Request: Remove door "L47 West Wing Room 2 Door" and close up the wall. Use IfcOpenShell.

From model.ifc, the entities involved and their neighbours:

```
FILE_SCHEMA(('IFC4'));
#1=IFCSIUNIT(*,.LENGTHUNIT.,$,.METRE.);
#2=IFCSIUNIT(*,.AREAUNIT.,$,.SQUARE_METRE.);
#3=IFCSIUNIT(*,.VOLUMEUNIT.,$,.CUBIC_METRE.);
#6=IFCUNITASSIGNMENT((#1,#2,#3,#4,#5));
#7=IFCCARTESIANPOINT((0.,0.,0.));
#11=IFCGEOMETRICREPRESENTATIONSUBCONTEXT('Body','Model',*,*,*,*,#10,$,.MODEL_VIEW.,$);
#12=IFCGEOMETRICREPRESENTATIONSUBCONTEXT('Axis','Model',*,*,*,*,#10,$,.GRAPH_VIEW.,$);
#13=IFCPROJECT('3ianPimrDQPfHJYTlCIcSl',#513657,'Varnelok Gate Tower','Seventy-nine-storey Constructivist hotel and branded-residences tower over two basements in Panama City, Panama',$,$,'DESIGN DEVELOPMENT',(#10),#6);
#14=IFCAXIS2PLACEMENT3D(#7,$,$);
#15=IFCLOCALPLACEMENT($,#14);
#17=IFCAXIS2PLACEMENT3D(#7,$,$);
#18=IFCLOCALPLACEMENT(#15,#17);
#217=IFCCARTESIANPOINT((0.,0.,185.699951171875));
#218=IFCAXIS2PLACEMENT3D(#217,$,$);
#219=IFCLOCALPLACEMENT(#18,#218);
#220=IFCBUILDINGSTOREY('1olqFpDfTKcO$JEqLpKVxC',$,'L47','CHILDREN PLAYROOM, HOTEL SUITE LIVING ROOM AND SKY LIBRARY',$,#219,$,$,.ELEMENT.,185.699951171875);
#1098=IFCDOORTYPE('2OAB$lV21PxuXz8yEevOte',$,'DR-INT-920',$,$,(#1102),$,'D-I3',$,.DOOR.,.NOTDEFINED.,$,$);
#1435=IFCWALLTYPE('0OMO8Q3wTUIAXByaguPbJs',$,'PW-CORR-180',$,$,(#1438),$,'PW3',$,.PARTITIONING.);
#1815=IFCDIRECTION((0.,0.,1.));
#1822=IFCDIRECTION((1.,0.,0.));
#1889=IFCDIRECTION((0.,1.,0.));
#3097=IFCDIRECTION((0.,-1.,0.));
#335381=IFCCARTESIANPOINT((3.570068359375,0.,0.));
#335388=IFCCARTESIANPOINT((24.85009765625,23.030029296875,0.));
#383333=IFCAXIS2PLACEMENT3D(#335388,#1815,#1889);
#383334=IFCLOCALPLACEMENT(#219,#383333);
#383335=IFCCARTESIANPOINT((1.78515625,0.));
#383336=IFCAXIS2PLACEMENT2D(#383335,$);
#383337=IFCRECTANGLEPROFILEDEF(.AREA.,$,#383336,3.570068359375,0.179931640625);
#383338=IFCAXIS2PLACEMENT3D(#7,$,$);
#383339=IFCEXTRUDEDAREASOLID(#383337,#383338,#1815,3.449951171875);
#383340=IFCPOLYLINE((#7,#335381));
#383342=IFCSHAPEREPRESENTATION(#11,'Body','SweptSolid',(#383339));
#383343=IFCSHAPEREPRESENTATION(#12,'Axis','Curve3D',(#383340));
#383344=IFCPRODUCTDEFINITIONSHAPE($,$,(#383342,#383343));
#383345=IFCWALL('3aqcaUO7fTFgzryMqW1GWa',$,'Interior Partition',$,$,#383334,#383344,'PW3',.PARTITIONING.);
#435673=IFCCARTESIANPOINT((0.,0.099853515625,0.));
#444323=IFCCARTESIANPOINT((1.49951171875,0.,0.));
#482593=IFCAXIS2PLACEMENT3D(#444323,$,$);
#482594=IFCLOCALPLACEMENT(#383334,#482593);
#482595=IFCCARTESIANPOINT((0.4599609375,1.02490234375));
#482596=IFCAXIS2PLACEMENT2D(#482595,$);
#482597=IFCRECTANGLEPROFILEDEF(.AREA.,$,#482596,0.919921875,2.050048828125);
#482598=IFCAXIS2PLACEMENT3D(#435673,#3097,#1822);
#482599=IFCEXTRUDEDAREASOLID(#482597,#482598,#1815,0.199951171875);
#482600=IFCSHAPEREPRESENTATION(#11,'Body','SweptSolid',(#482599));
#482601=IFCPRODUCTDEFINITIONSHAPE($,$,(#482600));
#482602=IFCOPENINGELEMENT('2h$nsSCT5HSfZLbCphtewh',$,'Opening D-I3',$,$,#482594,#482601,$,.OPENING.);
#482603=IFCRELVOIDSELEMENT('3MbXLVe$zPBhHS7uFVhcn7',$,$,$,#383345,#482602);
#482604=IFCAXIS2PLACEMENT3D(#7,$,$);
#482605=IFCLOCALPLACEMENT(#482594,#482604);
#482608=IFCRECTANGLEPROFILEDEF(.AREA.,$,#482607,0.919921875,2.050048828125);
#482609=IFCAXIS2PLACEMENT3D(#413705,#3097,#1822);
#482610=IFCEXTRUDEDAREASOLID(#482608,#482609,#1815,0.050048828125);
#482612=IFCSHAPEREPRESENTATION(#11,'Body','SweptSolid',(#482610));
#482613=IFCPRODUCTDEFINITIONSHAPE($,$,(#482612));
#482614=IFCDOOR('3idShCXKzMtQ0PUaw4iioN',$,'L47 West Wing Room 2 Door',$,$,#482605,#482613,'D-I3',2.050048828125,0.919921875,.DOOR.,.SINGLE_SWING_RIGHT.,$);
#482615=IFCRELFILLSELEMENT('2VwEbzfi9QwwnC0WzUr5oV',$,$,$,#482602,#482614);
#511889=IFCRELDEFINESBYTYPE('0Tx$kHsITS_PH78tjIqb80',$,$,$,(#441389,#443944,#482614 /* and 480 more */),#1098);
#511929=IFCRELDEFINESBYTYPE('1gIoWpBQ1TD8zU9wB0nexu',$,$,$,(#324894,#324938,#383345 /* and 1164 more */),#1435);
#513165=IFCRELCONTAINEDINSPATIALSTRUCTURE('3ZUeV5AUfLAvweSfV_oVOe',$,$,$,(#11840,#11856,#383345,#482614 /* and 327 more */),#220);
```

```python
import ifcopenshell
import ifcopenshell.api.feature
import ifcopenshell.api.root
import ifcopenshell.geom
import ifcopenshell.util.shape

model = ifcopenshell.open("model.ifc")
settings = ifcopenshell.geom.settings()


def volume(element):
    """Net volume in cubic metres, openings subtracted."""
    shape = ifcopenshell.geom.create_shape(settings, element)
    return ifcopenshell.util.shape.get_volume(shape.geometry)


door = model.by_guid("3idShCXKzMtQ0PUaw4iioN")
opening = door.FillsVoids[0].RelatingOpeningElement
wall = opening.VoidsElements[0].RelatingBuildingElement
before = volume(wall)

ifcopenshell.api.root.remove_product(model, product=door)
ifcopenshell.api.feature.remove_feature(model, feature=opening)

after = volume(wall)

print(f"wall volume {before:.3f} -> {after:.3f} m3")

model.write("model-out.ifc")
```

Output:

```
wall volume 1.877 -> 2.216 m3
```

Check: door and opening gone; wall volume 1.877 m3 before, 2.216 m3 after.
